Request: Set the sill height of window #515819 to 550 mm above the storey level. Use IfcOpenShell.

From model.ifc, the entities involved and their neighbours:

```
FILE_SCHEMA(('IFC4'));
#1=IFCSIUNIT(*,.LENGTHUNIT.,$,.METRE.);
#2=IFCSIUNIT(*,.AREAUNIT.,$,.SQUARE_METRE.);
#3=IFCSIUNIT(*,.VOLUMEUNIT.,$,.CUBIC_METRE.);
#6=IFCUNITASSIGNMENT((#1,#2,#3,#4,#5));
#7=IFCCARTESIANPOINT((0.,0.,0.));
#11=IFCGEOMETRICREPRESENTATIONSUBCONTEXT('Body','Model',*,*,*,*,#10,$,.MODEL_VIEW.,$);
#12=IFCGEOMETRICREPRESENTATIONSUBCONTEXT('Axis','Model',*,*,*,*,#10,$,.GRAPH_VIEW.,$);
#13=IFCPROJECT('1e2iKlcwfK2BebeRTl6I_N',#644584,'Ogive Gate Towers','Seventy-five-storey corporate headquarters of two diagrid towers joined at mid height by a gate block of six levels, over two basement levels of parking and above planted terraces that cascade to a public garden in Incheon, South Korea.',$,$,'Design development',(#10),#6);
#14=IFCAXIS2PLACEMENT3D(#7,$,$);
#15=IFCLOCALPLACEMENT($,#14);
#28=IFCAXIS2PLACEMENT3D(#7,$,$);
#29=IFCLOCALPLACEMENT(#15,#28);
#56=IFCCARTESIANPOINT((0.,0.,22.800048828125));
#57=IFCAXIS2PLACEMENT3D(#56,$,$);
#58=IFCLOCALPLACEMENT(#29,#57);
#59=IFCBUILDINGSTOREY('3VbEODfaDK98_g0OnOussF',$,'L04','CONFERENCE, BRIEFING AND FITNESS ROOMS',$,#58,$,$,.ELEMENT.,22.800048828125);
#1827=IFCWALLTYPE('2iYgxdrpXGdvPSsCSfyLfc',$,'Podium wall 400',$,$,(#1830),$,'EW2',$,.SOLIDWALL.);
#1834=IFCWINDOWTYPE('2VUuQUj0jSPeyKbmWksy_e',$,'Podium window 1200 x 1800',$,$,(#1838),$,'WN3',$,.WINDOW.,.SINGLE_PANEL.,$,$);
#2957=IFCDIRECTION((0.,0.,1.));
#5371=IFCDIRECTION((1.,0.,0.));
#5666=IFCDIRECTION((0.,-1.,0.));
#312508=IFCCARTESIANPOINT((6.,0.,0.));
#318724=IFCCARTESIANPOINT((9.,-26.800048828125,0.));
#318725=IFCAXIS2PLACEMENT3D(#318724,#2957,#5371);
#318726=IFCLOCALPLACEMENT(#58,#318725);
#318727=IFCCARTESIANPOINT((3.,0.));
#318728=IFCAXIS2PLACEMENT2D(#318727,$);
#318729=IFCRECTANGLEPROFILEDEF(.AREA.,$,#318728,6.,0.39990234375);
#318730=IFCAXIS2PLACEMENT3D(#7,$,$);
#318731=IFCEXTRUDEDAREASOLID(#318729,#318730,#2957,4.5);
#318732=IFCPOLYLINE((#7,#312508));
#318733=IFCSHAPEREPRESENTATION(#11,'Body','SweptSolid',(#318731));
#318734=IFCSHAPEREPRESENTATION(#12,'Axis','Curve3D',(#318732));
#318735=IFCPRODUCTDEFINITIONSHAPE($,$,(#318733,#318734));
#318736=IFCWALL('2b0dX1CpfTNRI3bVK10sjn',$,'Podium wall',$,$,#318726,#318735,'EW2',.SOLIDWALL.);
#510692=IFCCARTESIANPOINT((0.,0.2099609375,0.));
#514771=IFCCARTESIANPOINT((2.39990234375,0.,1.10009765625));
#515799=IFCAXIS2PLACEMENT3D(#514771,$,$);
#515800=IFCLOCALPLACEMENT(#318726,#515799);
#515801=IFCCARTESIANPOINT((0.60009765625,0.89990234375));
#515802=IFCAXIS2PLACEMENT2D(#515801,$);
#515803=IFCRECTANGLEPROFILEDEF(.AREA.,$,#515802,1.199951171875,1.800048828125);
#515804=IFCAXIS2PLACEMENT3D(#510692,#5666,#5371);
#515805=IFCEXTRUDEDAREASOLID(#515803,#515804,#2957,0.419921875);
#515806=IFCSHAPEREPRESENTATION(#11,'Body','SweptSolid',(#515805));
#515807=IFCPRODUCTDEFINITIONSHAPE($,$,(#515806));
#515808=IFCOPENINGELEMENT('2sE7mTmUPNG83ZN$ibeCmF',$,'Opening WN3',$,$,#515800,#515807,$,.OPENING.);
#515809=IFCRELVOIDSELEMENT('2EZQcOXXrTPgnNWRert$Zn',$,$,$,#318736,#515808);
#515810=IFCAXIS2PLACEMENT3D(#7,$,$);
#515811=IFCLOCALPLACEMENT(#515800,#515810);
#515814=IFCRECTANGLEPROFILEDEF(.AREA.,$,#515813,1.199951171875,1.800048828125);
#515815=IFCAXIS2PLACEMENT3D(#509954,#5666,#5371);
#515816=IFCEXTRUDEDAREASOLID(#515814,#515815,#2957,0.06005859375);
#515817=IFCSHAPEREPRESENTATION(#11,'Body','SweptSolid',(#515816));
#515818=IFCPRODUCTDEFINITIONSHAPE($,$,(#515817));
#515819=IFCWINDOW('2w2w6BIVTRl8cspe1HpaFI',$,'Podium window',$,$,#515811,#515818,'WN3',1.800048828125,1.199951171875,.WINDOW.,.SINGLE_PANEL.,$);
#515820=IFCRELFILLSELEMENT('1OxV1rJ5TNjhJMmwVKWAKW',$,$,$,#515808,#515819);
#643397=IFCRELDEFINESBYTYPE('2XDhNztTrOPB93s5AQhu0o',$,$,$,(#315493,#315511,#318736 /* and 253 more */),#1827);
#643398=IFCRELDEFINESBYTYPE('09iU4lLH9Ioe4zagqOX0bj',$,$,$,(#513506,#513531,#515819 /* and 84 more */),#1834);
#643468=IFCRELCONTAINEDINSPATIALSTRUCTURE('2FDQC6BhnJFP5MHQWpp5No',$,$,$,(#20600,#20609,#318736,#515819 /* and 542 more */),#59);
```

```python
import numpy as np
import ifcopenshell
import ifcopenshell.api.geometry
import ifcopenshell.geom
import ifcopenshell.util.element
import ifcopenshell.util.placement
import ifcopenshell.util.shape
import ifcopenshell.util.unit

model = ifcopenshell.open("model.ifc")
unit_scale = ifcopenshell.util.unit.calculate_unit_scale(model)

window = model.by_id(515819)
opening = window.FillsVoids[0].RelatingOpeningElement
storey = ifcopenshell.util.element.get_container(window, ifc_class="IfcBuildingStorey")
level = ifcopenshell.util.placement.get_local_placement(storey.ObjectPlacement)[2, 3]

# The opening's origin need not be at the sill, so measure its lowest point.
shape = ifcopenshell.geom.create_shape(ifcopenshell.geom.settings(), opening)
bottom = ifcopenshell.util.shape.get_shape_bottom_elevation(shape, shape.geometry) / unit_scale
dz = level + 0.55 / unit_scale - bottom

shift = np.array([0.0, 0.0, dz])
# The window is placed relative to its opening, so it follows when the opening moves.
matrix = ifcopenshell.util.placement.get_local_placement(opening.ObjectPlacement)
matrix[:3, 3] += shift
ifcopenshell.api.geometry.edit_object_placement(
    model, product=opening, matrix=matrix, is_si=False, should_transform_children=True
)

print(f"moved by {dz * unit_scale:+.3f} m")

model.write("model_rev.ifc")
```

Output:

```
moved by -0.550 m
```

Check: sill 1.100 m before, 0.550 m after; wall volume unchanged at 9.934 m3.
